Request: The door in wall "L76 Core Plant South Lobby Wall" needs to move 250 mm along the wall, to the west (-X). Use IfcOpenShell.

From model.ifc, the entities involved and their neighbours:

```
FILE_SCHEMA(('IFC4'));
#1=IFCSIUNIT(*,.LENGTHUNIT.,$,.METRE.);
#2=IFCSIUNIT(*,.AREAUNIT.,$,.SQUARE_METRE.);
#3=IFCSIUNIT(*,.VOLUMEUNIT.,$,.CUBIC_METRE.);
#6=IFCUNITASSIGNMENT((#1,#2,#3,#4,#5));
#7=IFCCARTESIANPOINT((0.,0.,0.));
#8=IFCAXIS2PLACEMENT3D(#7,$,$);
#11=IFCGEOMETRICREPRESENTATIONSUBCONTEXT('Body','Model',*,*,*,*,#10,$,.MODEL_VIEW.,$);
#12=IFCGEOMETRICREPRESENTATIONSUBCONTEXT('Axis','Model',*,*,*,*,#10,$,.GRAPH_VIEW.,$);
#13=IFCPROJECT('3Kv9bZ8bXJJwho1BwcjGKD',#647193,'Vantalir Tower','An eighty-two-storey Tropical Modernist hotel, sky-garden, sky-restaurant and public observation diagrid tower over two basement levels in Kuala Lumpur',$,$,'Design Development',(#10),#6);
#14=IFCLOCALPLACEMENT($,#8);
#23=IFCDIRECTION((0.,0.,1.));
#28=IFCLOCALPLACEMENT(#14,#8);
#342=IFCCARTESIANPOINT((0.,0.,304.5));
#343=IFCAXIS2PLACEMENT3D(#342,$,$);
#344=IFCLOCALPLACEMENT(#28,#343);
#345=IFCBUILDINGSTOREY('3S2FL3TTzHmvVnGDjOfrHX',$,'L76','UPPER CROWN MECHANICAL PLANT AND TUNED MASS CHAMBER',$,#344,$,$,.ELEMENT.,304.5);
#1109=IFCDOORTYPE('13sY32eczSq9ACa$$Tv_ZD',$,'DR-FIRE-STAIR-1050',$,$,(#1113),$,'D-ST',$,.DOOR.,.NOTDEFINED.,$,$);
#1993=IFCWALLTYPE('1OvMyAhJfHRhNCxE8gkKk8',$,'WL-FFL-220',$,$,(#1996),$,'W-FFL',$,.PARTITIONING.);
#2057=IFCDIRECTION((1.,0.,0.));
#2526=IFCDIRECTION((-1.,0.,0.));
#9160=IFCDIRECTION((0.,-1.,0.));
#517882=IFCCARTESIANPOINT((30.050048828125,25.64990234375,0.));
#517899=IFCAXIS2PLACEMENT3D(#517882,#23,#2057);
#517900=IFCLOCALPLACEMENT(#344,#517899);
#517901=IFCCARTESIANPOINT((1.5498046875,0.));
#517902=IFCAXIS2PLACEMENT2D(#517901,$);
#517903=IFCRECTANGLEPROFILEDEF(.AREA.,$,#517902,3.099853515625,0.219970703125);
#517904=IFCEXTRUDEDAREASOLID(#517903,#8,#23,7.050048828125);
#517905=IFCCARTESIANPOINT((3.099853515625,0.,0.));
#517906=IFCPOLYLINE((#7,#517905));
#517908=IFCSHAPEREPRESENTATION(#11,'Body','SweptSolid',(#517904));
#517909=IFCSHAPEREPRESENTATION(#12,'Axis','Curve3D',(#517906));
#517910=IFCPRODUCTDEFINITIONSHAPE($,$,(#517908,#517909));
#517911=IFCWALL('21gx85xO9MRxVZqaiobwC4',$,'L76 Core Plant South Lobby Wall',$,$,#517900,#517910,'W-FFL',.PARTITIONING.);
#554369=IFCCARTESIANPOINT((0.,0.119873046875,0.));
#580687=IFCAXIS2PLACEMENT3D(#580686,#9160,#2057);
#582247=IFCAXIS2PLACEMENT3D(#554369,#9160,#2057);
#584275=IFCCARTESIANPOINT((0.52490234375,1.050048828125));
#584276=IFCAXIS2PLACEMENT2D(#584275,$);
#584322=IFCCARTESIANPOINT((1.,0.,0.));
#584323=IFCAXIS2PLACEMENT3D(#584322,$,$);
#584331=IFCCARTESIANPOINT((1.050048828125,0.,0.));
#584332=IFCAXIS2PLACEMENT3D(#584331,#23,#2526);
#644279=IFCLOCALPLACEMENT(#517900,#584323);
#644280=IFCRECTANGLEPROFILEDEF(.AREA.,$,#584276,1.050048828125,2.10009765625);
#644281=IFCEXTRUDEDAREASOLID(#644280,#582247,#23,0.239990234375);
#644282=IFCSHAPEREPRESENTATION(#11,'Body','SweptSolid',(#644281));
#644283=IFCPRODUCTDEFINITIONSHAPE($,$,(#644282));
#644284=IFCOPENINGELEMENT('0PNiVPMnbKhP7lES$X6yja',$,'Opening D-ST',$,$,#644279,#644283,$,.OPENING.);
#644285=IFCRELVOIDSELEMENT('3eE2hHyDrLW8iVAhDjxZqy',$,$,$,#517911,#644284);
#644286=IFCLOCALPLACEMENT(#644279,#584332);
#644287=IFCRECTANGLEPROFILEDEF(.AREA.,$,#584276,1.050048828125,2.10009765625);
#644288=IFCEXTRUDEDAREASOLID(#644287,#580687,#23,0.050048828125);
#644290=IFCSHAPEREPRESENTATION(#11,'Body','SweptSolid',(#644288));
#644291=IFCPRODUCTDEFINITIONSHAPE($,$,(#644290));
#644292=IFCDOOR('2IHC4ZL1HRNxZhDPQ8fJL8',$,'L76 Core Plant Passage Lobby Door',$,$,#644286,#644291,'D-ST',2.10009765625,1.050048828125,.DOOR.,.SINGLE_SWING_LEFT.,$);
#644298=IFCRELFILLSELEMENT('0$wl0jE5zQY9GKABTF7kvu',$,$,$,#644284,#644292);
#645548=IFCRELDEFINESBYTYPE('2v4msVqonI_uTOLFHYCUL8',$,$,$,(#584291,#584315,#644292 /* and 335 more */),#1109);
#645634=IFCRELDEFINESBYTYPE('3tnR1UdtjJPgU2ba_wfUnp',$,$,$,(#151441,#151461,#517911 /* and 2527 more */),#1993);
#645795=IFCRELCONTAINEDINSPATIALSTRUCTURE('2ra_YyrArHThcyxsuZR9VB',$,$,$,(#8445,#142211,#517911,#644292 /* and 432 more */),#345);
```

```python
import ifcopenshell
import ifcopenshell.api.geometry
import ifcopenshell.util.placement

model = ifcopenshell.open("model.ifc")

door = model.by_guid("2IHC4ZL1HRNxZhDPQ8fJL8")
opening = door.FillsVoids[0].RelatingOpeningElement
wall = opening.VoidsElements[0].RelatingBuildingElement

wall_matrix = ifcopenshell.util.placement.get_local_placement(wall.ObjectPlacement)
shift = wall_matrix[:3, 0] * -0.25
before = ifcopenshell.util.placement.get_local_placement(door.ObjectPlacement)[:3, 3].copy()

# The door is placed relative to its opening, so it follows when the opening moves.
matrix = ifcopenshell.util.placement.get_local_placement(opening.ObjectPlacement)
matrix[:3, 3] += shift
ifcopenshell.api.geometry.edit_object_placement(
    model, product=opening, matrix=matrix, is_si=False, should_transform_children=True
)

after = ifcopenshell.util.placement.get_local_placement(door.ObjectPlacement)[:3, 3]
print("door moved by", (after - before).round(3) + 0.0)

model.write("model_rev.ifc")
```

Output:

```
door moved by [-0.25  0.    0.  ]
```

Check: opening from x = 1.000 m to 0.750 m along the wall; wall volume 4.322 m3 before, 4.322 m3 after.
